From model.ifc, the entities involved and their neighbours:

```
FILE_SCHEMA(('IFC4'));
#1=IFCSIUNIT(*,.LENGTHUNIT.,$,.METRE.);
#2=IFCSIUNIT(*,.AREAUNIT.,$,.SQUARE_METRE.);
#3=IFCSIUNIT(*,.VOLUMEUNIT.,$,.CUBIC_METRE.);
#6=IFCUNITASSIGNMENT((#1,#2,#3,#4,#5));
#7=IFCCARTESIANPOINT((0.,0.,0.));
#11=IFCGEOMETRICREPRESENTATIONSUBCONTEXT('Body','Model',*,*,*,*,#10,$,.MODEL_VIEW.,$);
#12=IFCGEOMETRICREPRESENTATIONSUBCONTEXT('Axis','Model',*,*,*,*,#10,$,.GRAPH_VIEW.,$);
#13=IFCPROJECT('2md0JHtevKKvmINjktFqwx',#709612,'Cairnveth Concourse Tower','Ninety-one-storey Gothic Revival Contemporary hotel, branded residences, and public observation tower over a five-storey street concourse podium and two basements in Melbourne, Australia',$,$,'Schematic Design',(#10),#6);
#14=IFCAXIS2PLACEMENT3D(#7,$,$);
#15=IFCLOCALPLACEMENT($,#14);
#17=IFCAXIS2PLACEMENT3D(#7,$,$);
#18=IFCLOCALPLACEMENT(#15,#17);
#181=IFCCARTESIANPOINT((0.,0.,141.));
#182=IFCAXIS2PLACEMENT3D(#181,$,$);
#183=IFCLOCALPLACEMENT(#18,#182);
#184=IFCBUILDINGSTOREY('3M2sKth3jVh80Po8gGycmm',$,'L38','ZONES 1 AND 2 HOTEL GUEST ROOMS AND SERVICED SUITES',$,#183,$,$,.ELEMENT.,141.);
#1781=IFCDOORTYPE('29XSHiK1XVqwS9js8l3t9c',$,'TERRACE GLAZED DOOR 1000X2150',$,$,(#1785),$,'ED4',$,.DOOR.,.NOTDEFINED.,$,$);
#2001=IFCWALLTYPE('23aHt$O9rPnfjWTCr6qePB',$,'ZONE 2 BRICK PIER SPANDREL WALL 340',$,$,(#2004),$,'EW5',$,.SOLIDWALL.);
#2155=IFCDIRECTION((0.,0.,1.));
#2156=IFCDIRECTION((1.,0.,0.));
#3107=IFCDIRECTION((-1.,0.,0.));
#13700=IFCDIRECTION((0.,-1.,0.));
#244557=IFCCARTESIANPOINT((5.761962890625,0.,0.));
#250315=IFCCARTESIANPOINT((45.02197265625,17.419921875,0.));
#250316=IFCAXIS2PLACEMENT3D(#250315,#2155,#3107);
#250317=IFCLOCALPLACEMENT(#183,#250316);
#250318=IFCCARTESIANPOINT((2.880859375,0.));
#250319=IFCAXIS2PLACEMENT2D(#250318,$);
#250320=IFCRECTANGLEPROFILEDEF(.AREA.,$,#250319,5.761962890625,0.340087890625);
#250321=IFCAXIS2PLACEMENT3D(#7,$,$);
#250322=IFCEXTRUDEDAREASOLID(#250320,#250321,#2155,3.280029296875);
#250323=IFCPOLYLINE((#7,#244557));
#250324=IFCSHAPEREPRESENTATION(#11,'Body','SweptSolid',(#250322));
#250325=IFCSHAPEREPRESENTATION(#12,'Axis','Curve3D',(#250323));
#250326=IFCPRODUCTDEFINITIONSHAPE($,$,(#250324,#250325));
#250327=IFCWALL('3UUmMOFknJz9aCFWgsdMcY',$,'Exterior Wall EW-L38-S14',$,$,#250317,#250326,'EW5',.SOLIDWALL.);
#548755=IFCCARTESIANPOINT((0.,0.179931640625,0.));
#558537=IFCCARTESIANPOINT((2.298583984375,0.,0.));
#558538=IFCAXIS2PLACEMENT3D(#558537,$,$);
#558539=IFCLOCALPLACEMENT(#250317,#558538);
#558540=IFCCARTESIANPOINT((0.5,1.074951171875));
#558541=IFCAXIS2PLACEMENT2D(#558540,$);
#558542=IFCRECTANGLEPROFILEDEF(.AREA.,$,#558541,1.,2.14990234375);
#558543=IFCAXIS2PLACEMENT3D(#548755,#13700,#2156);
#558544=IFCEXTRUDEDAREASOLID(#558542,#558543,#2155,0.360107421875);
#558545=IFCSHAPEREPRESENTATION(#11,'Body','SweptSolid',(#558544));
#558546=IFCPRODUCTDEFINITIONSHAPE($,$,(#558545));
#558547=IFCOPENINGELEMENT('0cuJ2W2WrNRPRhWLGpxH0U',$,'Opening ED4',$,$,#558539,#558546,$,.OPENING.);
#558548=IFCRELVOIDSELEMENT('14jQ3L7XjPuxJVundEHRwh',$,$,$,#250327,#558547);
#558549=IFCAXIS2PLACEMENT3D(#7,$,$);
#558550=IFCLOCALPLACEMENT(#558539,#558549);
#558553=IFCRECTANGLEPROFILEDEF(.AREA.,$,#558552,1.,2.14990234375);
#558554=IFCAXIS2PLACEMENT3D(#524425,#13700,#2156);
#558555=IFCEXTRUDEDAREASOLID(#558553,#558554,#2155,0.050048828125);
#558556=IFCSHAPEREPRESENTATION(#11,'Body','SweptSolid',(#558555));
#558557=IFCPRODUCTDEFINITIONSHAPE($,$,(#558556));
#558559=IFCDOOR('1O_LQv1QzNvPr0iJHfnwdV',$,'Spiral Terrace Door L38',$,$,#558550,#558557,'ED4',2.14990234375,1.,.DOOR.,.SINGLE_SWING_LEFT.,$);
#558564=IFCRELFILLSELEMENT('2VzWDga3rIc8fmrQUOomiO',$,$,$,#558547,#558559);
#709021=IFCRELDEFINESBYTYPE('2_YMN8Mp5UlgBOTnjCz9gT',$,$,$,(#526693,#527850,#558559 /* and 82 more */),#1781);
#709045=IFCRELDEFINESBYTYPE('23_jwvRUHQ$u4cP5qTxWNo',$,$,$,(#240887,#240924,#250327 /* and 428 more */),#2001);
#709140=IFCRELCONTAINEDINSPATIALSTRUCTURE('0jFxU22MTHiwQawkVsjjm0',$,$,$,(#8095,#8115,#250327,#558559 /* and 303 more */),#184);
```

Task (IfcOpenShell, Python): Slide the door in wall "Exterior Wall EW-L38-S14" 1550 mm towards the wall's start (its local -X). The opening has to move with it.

```python
import ifcopenshell
import ifcopenshell.api.geometry
import ifcopenshell.util.placement
import ifcopenshell.util.unit

model = ifcopenshell.open("model.ifc")
unit_scale = ifcopenshell.util.unit.calculate_unit_scale(model)

door = model.by_guid("1O_LQv1QzNvPr0iJHfnwdV")
opening = door.FillsVoids[0].RelatingOpeningElement
wall = opening.VoidsElements[0].RelatingBuildingElement

wall_matrix = ifcopenshell.util.placement.get_local_placement(wall.ObjectPlacement)
shift = wall_matrix[:3, 0] * -1.55 / unit_scale
before = ifcopenshell.util.placement.get_local_placement(door.ObjectPlacement)[:3, 3].copy()

# The door is placed relative to its opening, so it follows when the opening moves.
matrix = ifcopenshell.util.placement.get_local_placement(opening.ObjectPlacement)
matrix[:3, 3] += shift
ifcopenshell.api.geometry.edit_object_placement(
    model, product=opening, matrix=matrix, is_si=False, should_transform_children=True
)

after = ifcopenshell.util.placement.get_local_placement(door.ObjectPlacement)[:3, 3]
print("door moved by", (after - before).round(3) + 0.0)

model.write("model-out.ifc")
```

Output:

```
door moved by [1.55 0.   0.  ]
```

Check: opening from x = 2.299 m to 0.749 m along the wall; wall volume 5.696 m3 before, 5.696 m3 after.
